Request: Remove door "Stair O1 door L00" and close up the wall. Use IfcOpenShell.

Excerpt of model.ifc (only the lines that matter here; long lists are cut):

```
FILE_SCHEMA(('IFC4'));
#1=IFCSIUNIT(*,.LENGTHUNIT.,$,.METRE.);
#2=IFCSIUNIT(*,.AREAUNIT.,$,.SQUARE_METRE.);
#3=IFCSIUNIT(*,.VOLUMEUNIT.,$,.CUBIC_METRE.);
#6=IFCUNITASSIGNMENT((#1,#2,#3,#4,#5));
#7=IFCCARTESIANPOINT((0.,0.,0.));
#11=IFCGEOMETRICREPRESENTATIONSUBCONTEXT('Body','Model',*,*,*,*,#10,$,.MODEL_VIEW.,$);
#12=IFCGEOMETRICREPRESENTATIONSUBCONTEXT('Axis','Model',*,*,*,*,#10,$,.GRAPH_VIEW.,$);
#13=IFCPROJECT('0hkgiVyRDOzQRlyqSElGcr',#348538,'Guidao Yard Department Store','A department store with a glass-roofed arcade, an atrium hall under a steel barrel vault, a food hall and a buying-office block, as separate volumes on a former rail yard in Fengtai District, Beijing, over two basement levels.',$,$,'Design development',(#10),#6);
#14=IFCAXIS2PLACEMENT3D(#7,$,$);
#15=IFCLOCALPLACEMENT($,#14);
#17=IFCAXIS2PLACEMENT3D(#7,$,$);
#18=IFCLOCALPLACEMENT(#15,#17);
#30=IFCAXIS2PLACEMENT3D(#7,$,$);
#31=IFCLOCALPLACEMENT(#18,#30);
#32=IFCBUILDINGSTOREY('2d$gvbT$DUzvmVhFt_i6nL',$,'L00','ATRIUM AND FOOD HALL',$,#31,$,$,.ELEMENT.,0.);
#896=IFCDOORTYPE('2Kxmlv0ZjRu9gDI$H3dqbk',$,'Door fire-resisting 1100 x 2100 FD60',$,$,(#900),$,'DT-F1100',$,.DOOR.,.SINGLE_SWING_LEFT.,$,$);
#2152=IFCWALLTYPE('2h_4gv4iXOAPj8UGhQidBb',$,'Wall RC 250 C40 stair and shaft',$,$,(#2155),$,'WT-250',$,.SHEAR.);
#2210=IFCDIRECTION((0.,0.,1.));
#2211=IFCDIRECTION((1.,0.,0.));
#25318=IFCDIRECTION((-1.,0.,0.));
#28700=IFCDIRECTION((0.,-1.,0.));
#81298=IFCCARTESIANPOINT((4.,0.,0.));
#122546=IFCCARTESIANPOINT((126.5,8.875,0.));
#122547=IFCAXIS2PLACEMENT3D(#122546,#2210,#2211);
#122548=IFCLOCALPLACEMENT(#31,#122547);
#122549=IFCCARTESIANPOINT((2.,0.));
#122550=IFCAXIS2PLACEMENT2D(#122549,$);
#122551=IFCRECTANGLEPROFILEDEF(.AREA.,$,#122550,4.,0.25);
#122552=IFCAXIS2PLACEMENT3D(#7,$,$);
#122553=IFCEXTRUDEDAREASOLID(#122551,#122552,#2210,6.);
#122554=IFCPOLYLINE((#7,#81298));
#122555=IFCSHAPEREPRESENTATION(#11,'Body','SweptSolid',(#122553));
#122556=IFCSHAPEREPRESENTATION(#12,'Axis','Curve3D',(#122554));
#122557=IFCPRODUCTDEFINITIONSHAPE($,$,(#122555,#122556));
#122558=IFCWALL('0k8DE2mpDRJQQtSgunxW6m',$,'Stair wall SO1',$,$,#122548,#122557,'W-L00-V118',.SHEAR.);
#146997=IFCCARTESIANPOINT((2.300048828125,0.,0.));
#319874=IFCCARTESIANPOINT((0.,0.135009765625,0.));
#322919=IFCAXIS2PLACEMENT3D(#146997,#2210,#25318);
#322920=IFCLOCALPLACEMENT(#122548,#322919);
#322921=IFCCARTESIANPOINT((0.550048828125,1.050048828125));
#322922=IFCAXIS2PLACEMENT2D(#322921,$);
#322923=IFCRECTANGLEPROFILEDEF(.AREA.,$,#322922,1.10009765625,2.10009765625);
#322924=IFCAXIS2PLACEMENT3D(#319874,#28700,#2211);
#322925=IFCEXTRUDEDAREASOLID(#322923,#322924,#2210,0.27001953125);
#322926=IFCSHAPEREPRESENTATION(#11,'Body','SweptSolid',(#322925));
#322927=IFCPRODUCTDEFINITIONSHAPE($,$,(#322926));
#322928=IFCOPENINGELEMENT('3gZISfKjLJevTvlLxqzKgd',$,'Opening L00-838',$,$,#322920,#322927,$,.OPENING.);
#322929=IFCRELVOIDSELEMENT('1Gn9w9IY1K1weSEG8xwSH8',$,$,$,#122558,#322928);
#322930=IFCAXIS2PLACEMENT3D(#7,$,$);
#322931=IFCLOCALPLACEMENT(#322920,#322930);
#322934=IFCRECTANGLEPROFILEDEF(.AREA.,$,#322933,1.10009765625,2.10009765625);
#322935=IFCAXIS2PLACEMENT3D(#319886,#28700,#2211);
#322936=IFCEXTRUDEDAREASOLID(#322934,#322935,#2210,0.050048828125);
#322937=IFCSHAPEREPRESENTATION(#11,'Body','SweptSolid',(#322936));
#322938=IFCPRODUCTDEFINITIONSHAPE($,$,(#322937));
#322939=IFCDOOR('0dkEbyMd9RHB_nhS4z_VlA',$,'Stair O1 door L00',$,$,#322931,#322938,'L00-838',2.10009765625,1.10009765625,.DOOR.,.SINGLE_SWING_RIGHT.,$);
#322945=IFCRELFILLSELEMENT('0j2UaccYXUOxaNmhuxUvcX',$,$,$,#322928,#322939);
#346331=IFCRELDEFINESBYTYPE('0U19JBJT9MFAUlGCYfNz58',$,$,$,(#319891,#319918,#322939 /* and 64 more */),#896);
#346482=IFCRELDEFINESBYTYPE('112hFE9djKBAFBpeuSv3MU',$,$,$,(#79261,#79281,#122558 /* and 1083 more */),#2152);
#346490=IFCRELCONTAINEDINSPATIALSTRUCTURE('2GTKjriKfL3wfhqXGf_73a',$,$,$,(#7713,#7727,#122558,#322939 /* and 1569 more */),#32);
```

```python
import ifcopenshell
import ifcopenshell.api.feature
import ifcopenshell.api.root
import ifcopenshell.geom
import ifcopenshell.util.shape

model = ifcopenshell.open("model.ifc")
settings = ifcopenshell.geom.settings()


def volume(element):
    """Net volume in cubic metres, openings subtracted."""
    shape = ifcopenshell.geom.create_shape(settings, element)
    return ifcopenshell.util.shape.get_volume(shape.geometry)


door = model.by_id(322939)
opening = door.FillsVoids[0].RelatingOpeningElement
wall = opening.VoidsElements[0].RelatingBuildingElement
before = volume(wall)

ifcopenshell.api.root.remove_product(model, product=door)
ifcopenshell.api.feature.remove_feature(model, feature=opening)

after = volume(wall)

print(f"wall volume {before:.3f} -> {after:.3f} m3")

model.write("model_v2.ifc")
```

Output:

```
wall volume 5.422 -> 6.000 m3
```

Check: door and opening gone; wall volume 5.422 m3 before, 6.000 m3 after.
